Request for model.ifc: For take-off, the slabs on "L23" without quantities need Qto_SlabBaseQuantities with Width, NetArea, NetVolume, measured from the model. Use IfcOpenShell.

First a look at what the model holds.

```python
import ifcopenshell
import ifcopenshell.util.element
import ifcopenshell.util.unit

model = ifcopenshell.open("model.ifc")
print(model.schema)
for unit_type in ("LENGTHUNIT", "AREAUNIT", "VOLUMEUNIT"):
    print(unit_type, ifcopenshell.util.unit.calculate_unit_scale(model, unit_type))
storey = next(s for s in model.by_type("IfcBuildingStorey") if s.Name == "L23")
slabs = [e for e in ifcopenshell.util.element.get_decomposition(storey) if e.is_a("IfcSlab")]
for e in sorted(slabs, key=lambda e: e.id()):
    print(e.id(), e.is_a(), e.Name, list(ifcopenshell.util.element.get_psets(e, qtos_only=True)), sep=" | ")
```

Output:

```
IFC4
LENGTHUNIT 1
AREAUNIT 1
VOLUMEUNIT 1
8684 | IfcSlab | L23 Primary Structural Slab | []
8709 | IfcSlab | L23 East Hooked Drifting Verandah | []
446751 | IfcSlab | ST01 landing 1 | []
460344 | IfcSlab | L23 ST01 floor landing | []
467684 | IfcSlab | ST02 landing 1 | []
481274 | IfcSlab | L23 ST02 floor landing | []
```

```python
import ifcopenshell
import ifcopenshell.api.pset
import ifcopenshell.geom
import ifcopenshell.util.element
import ifcopenshell.util.shape
import ifcopenshell.util.unit

model = ifcopenshell.open("model.ifc")
unit_scale = ifcopenshell.util.unit.calculate_unit_scale(model)
area_scale = ifcopenshell.util.unit.calculate_unit_scale(model, "AREAUNIT")
volume_scale = ifcopenshell.util.unit.calculate_unit_scale(model, "VOLUMEUNIT")
settings = ifcopenshell.geom.settings()

storey = next(s for s in model.by_type("IfcBuildingStorey") if s.Name == "L23")
slabs = [e for e in ifcopenshell.util.element.get_decomposition(storey) if e.is_a("IfcSlab")]

for e in sorted(slabs, key=lambda e: e.id()):
    if ifcopenshell.util.element.get_psets(e, qtos_only=True, should_inherit=False):
        continue
    # Geometry comes back in metres, in the element's own axes.
    shape = ifcopenshell.geom.create_shape(settings, e)
    values = {
        "Width": ifcopenshell.util.shape.get_z(shape.geometry) / unit_scale,
        "NetArea": ifcopenshell.util.shape.get_footprint_area(shape.geometry) / area_scale,
        "NetVolume": ifcopenshell.util.shape.get_volume(shape.geometry) / volume_scale,
    }
    qto = ifcopenshell.api.pset.add_qto(model, product=e, name="Qto_SlabBaseQuantities")
    ifcopenshell.api.pset.edit_qto(model, qto=qto, properties=values)
    print(e.id(), {k: round(v, 3) for k, v in values.items()})

model.write("model_updated.ifc")
```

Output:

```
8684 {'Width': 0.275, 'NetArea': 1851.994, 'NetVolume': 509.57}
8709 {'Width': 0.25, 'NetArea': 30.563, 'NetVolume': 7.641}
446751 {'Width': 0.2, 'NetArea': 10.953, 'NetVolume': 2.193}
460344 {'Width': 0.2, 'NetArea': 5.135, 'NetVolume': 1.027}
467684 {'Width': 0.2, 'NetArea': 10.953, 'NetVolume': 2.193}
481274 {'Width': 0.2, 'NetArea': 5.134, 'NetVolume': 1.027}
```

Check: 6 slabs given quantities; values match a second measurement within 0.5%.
